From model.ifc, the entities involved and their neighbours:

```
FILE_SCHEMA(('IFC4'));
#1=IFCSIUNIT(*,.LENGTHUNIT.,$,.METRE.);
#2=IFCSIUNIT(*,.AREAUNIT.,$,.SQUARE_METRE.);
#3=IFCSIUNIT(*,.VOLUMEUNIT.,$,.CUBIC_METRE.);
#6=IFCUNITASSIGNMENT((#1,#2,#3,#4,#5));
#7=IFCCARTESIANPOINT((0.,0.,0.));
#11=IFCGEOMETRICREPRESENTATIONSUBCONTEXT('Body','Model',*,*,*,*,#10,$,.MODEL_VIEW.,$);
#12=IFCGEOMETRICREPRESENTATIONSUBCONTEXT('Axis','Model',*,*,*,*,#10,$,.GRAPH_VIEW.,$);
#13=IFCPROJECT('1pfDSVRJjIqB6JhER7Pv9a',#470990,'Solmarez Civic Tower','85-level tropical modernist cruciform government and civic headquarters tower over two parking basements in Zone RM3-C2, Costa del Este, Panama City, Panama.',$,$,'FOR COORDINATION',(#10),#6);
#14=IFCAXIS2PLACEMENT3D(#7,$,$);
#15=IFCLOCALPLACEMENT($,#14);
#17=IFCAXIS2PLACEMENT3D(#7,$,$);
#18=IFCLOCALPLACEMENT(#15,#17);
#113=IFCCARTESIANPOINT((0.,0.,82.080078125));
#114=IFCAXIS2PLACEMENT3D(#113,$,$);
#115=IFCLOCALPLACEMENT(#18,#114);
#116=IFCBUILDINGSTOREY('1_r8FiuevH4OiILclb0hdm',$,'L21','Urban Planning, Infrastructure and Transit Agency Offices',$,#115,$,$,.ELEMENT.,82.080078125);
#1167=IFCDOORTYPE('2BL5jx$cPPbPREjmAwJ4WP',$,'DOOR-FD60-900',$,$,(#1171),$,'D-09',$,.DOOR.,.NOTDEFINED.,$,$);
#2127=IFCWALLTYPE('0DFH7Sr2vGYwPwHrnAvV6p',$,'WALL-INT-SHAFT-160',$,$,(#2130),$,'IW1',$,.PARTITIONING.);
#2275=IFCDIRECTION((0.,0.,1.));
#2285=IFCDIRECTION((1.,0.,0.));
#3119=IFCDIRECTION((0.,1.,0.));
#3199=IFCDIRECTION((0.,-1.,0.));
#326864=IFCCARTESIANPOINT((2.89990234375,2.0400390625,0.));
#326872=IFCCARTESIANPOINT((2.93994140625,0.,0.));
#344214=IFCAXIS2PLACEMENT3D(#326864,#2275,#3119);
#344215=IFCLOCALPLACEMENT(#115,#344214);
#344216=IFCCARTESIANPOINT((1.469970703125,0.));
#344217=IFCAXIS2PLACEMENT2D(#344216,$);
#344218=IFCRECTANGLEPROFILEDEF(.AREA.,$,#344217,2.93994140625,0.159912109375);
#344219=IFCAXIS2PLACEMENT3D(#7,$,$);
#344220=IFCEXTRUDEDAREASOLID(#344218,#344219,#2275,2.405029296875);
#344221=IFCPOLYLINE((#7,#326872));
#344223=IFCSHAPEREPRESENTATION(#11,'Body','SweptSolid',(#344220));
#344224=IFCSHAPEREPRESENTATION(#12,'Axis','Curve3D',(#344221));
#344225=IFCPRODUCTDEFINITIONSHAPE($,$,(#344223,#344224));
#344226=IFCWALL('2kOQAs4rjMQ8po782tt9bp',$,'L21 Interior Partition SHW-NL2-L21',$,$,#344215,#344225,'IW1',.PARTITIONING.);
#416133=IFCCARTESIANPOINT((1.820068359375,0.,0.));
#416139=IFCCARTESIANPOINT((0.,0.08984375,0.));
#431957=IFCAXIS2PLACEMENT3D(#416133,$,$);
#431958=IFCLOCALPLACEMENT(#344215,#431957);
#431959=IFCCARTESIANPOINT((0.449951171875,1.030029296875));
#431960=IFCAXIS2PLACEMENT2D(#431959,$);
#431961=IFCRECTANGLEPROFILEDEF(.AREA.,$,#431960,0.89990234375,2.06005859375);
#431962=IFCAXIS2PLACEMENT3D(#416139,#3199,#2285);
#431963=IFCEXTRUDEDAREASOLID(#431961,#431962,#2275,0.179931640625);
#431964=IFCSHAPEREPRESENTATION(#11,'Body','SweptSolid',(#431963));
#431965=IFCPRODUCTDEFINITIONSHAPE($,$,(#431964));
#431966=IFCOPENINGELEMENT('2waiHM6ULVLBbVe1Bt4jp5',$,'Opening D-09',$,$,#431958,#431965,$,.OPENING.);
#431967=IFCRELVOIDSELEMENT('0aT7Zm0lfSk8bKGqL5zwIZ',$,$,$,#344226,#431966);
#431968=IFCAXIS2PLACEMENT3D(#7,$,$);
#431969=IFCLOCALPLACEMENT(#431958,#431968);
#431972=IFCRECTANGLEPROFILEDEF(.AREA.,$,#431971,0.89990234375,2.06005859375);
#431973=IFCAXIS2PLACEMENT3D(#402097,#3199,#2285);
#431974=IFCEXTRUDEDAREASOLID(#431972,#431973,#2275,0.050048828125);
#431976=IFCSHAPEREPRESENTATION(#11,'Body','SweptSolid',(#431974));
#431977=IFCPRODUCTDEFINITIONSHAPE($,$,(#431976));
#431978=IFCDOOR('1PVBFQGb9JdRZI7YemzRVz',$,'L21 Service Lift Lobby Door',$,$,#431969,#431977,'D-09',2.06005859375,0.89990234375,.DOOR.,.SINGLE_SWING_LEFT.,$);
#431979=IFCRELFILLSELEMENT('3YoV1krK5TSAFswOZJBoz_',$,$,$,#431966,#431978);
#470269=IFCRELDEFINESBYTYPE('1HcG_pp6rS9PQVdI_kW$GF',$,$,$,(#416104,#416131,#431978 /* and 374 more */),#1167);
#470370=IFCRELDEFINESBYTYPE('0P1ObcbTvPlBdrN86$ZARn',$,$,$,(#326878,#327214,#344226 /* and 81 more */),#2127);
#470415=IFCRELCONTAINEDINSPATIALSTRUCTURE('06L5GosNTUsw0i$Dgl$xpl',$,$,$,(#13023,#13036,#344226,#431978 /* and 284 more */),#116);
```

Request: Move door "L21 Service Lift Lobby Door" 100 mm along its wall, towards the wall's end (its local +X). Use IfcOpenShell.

```python
import ifcopenshell
import ifcopenshell.api.geometry
import ifcopenshell.util.placement
import ifcopenshell.util.unit

model = ifcopenshell.open("model.ifc")
unit_scale = ifcopenshell.util.unit.calculate_unit_scale(model)

door = model.by_guid("1PVBFQGb9JdRZI7YemzRVz")
opening = door.FillsVoids[0].RelatingOpeningElement
wall = opening.VoidsElements[0].RelatingBuildingElement

wall_matrix = ifcopenshell.util.placement.get_local_placement(wall.ObjectPlacement)
shift = wall_matrix[:3, 0] * 0.1 / unit_scale
before = ifcopenshell.util.placement.get_local_placement(door.ObjectPlacement)[:3, 3].copy()

# The door is placed relative to its opening, so it follows when the opening moves.
matrix = ifcopenshell.util.placement.get_local_placement(opening.ObjectPlacement)
matrix[:3, 3] += shift
ifcopenshell.api.geometry.edit_object_placement(
    model, product=opening, matrix=matrix, is_si=False, should_transform_children=True
)

after = ifcopenshell.util.placement.get_local_placement(door.ObjectPlacement)[:3, 3]
print("door moved by", (after - before).round(3) + 0.0)

model.write("model_rev.ifc")
```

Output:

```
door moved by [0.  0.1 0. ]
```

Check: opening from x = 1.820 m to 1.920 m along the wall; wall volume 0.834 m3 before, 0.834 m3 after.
